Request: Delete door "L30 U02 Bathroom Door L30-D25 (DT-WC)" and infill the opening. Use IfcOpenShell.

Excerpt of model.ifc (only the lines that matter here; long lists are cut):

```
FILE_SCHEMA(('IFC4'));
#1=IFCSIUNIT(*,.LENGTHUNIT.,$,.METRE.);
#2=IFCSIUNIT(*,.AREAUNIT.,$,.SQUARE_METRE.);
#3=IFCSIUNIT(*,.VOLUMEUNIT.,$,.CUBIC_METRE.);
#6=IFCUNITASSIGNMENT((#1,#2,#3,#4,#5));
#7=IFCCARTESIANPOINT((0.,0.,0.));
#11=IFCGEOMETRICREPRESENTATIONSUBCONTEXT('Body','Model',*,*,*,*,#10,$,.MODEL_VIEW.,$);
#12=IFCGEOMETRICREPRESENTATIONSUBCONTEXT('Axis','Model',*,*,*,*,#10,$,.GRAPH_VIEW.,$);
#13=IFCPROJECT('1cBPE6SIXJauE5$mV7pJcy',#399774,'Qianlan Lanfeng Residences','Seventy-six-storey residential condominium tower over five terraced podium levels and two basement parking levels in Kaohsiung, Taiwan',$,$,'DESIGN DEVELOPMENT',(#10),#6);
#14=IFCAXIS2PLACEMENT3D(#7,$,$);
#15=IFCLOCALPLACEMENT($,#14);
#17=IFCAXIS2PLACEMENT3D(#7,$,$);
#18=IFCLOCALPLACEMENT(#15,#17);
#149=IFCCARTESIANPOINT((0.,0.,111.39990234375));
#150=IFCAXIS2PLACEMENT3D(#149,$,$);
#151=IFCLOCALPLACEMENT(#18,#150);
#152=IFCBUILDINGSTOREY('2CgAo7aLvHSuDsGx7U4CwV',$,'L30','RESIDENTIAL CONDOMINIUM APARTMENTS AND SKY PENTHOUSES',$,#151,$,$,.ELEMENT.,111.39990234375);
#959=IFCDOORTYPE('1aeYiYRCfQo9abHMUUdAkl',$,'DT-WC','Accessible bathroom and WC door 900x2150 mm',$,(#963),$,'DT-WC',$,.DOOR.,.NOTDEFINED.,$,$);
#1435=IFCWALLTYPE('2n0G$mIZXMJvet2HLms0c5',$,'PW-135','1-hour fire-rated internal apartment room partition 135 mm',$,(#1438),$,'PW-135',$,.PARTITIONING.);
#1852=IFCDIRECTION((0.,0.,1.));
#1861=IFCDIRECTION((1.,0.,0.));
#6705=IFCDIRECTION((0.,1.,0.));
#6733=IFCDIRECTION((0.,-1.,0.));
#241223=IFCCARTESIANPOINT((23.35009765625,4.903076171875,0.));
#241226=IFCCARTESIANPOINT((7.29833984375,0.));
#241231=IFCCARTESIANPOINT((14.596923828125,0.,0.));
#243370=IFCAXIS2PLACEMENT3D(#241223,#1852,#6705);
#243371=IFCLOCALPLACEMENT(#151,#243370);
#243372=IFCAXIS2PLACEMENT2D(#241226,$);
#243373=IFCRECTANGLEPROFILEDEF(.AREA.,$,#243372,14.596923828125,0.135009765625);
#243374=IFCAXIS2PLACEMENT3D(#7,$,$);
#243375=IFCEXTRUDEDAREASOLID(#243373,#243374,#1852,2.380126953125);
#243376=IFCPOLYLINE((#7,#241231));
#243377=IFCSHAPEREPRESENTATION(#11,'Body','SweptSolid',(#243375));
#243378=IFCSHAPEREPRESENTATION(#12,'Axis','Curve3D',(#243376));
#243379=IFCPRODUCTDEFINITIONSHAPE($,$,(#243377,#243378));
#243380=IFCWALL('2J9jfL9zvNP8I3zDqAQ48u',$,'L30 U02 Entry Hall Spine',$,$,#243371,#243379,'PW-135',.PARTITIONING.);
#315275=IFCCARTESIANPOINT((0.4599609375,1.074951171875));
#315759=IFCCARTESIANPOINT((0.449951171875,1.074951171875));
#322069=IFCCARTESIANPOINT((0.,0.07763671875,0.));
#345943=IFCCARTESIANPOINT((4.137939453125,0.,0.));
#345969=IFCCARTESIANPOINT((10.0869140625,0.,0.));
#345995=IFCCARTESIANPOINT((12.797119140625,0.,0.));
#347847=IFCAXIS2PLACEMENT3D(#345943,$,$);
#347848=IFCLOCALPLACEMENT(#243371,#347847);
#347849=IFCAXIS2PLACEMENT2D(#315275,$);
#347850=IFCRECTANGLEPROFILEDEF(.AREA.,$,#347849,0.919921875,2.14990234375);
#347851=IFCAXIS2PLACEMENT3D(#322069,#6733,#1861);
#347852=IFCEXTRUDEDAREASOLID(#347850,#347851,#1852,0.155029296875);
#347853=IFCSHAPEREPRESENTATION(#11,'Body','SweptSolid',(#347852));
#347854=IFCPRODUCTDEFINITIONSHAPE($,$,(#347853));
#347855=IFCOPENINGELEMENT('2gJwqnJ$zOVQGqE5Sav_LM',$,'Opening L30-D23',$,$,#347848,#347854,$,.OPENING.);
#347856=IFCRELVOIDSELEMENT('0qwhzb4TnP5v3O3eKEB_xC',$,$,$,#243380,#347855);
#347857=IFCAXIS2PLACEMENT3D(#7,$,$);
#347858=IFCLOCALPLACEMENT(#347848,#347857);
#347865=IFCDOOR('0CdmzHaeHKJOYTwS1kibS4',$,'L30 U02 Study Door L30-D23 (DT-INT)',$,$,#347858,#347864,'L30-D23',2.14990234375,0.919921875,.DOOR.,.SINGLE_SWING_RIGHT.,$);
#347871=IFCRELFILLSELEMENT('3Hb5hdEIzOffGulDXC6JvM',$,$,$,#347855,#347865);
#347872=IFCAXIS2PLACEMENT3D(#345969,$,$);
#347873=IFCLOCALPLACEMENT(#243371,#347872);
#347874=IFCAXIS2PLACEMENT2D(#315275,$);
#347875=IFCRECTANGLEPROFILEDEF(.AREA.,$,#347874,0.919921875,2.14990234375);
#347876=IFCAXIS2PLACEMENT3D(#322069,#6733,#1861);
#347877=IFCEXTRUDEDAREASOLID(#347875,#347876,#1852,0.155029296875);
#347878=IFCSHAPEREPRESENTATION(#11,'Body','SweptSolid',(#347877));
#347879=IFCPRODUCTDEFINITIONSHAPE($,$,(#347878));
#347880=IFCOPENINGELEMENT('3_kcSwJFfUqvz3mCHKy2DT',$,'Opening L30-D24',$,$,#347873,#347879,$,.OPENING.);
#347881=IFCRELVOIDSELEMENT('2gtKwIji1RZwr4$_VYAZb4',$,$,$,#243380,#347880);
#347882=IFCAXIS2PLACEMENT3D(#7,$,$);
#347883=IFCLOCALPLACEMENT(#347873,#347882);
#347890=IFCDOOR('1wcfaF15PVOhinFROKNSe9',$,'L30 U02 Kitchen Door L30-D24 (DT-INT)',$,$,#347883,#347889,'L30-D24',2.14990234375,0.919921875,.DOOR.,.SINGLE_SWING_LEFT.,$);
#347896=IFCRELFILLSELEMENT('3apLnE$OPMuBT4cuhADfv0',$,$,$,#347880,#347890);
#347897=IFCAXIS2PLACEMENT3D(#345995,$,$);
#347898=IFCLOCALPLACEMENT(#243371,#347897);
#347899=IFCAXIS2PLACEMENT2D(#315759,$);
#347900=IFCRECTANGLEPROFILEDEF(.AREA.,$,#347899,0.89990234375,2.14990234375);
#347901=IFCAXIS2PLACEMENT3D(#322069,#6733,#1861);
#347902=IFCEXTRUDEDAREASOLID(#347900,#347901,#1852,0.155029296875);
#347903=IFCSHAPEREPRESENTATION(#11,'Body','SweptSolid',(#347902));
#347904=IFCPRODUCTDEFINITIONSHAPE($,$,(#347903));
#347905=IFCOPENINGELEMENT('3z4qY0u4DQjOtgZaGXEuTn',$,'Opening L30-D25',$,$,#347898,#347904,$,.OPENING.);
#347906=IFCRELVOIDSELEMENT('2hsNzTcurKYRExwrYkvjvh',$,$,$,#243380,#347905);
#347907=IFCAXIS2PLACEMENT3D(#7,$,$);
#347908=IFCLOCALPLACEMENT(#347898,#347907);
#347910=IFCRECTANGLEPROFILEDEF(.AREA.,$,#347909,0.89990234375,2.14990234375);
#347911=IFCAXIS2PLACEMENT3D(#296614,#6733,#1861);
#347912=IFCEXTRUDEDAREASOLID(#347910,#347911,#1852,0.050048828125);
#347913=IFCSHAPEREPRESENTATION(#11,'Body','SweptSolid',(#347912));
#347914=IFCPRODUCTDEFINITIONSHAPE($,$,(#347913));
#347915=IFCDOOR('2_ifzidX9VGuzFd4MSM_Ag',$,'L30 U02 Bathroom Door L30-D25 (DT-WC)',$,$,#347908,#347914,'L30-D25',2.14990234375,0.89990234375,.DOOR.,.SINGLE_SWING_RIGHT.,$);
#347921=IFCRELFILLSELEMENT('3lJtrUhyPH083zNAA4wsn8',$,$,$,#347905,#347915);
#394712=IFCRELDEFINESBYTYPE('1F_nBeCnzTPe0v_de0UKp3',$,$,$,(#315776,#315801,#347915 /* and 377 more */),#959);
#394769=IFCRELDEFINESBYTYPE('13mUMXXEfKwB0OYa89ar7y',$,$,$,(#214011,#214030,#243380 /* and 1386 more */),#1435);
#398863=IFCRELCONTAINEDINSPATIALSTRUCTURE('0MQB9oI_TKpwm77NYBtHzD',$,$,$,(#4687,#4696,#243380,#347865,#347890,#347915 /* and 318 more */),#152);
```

```python
import ifcopenshell
import ifcopenshell.api.feature
import ifcopenshell.api.root
import ifcopenshell.geom
import ifcopenshell.util.shape

model = ifcopenshell.open("model.ifc")
settings = ifcopenshell.geom.settings()


def volume(element):
    """Net volume in cubic metres, openings subtracted."""
    shape = ifcopenshell.geom.create_shape(settings, element)
    return ifcopenshell.util.shape.get_volume(shape.geometry)


door = model.by_guid("2_ifzidX9VGuzFd4MSM_Ag")
opening = door.FillsVoids[0].RelatingOpeningElement
wall = opening.VoidsElements[0].RelatingBuildingElement
before = volume(wall)

ifcopenshell.api.root.remove_product(model, product=door)
ifcopenshell.api.feature.remove_feature(model, feature=opening)

after = volume(wall)

print(f"wall volume {before:.3f} -> {after:.3f} m3")

model.write("model_edited.ifc")
```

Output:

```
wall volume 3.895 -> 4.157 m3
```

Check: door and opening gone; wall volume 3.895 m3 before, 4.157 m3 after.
